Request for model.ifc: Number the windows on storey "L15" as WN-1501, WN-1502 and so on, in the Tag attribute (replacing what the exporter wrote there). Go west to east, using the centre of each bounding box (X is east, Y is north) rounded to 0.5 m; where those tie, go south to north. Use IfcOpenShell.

First a look at what the model holds.

```python
import ifcopenshell
import ifcopenshell.util.element
import ifcopenshell.util.placement

model = ifcopenshell.open("model.ifc")
print(model.schema)
storey = next(s for s in model.by_type("IfcBuildingStorey") if s.Name == "L15")
windows = [e for e in ifcopenshell.util.element.get_decomposition(storey) if e.is_a("IfcWindow")]
for e in sorted(windows, key=lambda e: e.id()):
    origin = ifcopenshell.util.placement.get_local_placement(e.ObjectPlacement)[:3, 3]
    print(e.id(), e.Tag, e.Name, origin.round(2) + 0.0, sep=" | ")
```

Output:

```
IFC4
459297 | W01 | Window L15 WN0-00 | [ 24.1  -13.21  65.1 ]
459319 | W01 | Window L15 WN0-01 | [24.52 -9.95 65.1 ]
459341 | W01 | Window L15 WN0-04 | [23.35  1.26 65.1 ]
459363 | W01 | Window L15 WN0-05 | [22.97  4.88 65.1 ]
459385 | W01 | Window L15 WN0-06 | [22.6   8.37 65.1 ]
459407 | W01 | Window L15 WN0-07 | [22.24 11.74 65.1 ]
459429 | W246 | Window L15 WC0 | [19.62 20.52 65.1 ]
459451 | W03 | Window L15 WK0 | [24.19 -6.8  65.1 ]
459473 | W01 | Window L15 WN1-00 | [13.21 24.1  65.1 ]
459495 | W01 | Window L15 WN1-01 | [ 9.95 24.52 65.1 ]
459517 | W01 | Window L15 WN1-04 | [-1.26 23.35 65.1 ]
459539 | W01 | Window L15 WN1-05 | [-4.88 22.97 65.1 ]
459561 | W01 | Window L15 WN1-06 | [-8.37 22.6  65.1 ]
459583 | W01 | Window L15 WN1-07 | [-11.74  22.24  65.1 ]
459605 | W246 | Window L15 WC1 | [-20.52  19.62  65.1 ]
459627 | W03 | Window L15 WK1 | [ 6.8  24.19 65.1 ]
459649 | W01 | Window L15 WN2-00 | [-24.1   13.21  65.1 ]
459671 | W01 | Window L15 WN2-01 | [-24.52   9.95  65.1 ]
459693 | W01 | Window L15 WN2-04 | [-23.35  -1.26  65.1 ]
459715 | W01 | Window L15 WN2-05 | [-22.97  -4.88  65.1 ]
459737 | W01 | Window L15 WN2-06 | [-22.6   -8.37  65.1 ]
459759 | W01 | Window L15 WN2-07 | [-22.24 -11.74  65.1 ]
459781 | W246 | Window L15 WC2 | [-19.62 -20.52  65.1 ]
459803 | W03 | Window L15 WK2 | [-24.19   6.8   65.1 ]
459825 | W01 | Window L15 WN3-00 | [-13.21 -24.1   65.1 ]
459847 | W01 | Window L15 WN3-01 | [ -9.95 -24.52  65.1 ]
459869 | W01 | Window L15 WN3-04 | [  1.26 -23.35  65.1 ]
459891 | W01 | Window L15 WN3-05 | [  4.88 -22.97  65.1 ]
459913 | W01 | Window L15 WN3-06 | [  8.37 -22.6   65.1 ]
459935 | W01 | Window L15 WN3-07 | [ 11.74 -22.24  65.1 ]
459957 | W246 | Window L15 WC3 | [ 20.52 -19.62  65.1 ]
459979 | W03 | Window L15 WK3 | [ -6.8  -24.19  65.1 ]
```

```python
import ifcopenshell
import ifcopenshell.geom
import ifcopenshell.util.element
import ifcopenshell.util.shape

model = ifcopenshell.open("model.ifc")
settings = ifcopenshell.geom.settings()
settings.set("use-world-coords", True)


def centre(element):
    shape = ifcopenshell.geom.create_shape(settings, element)
    return ifcopenshell.util.shape.get_bbox_centroid(shape.geometry)


storey = next(s for s in model.by_type("IfcBuildingStorey") if s.Name == "L15")
windows = [e for e in ifcopenshell.util.element.get_decomposition(storey) if e.is_a("IfcWindow")]

# Insertion points can sit at a corner or the storey origin, so sort by the geometry (in metres).
centres = {e: centre(e) for e in windows}
windows.sort(key=lambda e: (round(centres[e][0] / 0.5), centres[e][1]))

for i, e in enumerate(windows, start=1):
    number = f"WN-15{i:02d}"
    e.Tag = number
    print(e.id(), number)

model.write("model_v2.ifc")
```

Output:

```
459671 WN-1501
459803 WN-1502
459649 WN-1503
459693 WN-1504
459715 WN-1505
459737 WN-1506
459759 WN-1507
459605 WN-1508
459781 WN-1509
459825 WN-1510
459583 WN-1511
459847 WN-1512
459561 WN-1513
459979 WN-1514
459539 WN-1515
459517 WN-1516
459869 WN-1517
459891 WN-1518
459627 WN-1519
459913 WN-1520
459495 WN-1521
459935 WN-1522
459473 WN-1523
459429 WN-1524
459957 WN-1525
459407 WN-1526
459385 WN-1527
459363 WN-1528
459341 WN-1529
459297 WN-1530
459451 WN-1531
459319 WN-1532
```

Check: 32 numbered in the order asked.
